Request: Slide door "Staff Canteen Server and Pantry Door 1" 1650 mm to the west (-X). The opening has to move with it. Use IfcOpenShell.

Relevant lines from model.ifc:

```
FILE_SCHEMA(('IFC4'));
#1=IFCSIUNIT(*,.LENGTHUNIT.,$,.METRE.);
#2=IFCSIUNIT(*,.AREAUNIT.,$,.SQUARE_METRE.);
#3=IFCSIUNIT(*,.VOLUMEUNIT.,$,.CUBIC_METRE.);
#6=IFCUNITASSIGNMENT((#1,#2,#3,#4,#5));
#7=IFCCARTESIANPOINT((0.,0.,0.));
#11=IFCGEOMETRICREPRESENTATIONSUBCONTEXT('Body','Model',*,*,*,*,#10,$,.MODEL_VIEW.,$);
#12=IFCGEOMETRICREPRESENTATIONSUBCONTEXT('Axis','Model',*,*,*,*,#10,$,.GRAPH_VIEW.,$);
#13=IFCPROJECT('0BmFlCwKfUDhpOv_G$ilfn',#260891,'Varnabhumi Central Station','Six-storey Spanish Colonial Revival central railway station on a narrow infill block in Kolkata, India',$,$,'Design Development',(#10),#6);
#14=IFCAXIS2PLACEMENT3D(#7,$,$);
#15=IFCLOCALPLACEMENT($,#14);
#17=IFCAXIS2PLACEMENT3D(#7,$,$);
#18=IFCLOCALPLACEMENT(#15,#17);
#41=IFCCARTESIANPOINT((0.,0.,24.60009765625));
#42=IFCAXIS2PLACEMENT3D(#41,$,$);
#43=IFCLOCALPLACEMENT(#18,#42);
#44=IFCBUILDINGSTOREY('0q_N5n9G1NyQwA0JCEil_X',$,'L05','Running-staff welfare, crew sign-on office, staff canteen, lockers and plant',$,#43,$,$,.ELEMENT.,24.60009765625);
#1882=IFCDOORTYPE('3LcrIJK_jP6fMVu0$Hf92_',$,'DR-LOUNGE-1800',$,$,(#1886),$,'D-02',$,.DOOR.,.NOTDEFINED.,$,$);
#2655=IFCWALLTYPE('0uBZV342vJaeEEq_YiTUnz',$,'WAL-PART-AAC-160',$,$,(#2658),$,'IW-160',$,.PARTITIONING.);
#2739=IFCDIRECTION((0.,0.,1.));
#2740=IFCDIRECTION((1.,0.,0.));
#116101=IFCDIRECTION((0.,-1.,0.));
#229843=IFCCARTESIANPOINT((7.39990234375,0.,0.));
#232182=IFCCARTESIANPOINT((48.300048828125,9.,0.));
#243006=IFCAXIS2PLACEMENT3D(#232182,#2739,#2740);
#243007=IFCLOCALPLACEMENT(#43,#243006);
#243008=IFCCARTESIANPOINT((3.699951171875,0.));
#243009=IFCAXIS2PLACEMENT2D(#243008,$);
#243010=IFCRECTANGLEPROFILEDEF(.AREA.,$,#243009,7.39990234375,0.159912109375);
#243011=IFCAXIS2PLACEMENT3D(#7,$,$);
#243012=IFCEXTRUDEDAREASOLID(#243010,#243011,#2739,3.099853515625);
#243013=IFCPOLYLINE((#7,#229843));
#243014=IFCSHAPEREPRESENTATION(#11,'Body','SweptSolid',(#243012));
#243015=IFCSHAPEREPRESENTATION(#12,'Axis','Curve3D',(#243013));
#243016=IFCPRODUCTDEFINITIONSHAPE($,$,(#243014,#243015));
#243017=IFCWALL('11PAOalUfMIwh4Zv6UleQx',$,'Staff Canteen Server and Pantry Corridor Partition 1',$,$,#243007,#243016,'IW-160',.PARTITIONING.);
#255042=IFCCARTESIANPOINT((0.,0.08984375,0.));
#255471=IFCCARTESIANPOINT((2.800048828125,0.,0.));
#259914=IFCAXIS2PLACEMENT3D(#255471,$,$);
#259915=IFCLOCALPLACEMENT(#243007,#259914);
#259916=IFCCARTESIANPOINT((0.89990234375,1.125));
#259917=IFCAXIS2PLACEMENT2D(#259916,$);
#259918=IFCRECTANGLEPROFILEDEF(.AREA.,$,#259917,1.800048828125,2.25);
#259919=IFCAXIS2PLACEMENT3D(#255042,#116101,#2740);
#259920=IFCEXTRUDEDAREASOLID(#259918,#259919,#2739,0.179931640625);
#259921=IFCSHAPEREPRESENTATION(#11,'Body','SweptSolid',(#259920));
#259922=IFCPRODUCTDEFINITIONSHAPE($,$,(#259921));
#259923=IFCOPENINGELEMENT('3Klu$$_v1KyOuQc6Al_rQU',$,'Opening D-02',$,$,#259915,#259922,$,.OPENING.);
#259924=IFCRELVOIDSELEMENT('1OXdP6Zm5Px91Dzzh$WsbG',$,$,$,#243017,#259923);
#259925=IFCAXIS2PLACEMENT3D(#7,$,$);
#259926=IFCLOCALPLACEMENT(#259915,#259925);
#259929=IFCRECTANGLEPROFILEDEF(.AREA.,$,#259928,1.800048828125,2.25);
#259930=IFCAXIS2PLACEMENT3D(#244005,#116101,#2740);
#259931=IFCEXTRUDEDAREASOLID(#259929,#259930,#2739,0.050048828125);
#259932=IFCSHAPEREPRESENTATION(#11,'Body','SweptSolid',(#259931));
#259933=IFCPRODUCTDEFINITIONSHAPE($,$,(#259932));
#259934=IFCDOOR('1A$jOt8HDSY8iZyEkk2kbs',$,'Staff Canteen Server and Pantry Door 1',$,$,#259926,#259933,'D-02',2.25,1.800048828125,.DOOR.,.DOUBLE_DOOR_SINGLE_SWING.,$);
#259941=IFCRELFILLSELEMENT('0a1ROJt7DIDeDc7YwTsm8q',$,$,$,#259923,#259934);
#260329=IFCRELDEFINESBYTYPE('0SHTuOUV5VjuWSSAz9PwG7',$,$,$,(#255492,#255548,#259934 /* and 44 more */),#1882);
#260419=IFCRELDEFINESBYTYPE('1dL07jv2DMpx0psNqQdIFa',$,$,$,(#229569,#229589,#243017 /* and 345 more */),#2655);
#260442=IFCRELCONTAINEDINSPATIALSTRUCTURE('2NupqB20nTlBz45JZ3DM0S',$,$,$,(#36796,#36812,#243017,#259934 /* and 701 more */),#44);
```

```python
import ifcopenshell
import ifcopenshell.api.geometry
import ifcopenshell.util.placement
import ifcopenshell.util.unit

model = ifcopenshell.open("model.ifc")
unit_scale = ifcopenshell.util.unit.calculate_unit_scale(model)

door = model.by_id(259934)
opening = door.FillsVoids[0].RelatingOpeningElement
wall = opening.VoidsElements[0].RelatingBuildingElement

wall_matrix = ifcopenshell.util.placement.get_local_placement(wall.ObjectPlacement)
shift = wall_matrix[:3, 0] * -1.65 / unit_scale
before = ifcopenshell.util.placement.get_local_placement(door.ObjectPlacement)[:3, 3].copy()

# The door is placed relative to its opening, so it follows when the opening moves.
matrix = ifcopenshell.util.placement.get_local_placement(opening.ObjectPlacement)
matrix[:3, 3] += shift
ifcopenshell.api.geometry.edit_object_placement(
    model, product=opening, matrix=matrix, is_si=False, should_transform_children=True
)

after = ifcopenshell.util.placement.get_local_placement(door.ObjectPlacement)[:3, 3]
print("door moved by", (after - before).round(3) + 0.0)

model.write("model_edited.ifc")
```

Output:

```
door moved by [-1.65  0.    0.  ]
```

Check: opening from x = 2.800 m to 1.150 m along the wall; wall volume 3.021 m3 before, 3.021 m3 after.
